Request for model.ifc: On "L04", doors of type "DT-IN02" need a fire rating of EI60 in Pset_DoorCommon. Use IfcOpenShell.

First a look at what the model holds.

```python
import ifcopenshell
import ifcopenshell.util.element

model = ifcopenshell.open("model.ifc")
print(model.schema)
storey = next(s for s in model.by_type("IfcBuildingStorey") if s.Name == "L04")
doors = [e for e in ifcopenshell.util.element.get_decomposition(storey) if e.is_a("IfcDoor")]
seen = {}
for e in doors:
    element_type = ifcopenshell.util.element.get_type(e)
    key = (element_type.Name if element_type != e and element_type else None, ifcopenshell.util.element.get_pset(e, "Pset_DoorCommon", "FireRating"))
    seen[key] = seen.get(key, 0) + 1
for (name, value), count in sorted(seen.items(), key=str):
    print(count, "x", name, "|", value)
```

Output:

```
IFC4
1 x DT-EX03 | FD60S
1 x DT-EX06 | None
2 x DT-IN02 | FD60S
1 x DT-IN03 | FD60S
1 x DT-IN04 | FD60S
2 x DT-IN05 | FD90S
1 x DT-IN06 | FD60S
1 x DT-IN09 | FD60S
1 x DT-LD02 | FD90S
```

```python
import ifcopenshell
import ifcopenshell.api.pset
import ifcopenshell.util.element

model = ifcopenshell.open("model.ifc")

storey = next(s for s in model.by_type("IfcBuildingStorey") if s.Name == "L04")
doors = [e for e in ifcopenshell.util.element.get_decomposition(storey) if e.is_a("IfcDoor")]

count = 0
for e in doors:
    element_type = ifcopenshell.util.element.get_type(e)
    if element_type in (None, e) or element_type.Name != "DT-IN02":
        continue
    # add_pset returns the element's existing set when there is one.
    pset = ifcopenshell.api.pset.add_pset(model, product=e, name="Pset_DoorCommon")
    ifcopenshell.api.pset.edit_pset(model, pset=pset, properties={"FireRating": "EI60"})
    count += 1

print(count, "doors updated")

model.write("model_edited.ifc")
```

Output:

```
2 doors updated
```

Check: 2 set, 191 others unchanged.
